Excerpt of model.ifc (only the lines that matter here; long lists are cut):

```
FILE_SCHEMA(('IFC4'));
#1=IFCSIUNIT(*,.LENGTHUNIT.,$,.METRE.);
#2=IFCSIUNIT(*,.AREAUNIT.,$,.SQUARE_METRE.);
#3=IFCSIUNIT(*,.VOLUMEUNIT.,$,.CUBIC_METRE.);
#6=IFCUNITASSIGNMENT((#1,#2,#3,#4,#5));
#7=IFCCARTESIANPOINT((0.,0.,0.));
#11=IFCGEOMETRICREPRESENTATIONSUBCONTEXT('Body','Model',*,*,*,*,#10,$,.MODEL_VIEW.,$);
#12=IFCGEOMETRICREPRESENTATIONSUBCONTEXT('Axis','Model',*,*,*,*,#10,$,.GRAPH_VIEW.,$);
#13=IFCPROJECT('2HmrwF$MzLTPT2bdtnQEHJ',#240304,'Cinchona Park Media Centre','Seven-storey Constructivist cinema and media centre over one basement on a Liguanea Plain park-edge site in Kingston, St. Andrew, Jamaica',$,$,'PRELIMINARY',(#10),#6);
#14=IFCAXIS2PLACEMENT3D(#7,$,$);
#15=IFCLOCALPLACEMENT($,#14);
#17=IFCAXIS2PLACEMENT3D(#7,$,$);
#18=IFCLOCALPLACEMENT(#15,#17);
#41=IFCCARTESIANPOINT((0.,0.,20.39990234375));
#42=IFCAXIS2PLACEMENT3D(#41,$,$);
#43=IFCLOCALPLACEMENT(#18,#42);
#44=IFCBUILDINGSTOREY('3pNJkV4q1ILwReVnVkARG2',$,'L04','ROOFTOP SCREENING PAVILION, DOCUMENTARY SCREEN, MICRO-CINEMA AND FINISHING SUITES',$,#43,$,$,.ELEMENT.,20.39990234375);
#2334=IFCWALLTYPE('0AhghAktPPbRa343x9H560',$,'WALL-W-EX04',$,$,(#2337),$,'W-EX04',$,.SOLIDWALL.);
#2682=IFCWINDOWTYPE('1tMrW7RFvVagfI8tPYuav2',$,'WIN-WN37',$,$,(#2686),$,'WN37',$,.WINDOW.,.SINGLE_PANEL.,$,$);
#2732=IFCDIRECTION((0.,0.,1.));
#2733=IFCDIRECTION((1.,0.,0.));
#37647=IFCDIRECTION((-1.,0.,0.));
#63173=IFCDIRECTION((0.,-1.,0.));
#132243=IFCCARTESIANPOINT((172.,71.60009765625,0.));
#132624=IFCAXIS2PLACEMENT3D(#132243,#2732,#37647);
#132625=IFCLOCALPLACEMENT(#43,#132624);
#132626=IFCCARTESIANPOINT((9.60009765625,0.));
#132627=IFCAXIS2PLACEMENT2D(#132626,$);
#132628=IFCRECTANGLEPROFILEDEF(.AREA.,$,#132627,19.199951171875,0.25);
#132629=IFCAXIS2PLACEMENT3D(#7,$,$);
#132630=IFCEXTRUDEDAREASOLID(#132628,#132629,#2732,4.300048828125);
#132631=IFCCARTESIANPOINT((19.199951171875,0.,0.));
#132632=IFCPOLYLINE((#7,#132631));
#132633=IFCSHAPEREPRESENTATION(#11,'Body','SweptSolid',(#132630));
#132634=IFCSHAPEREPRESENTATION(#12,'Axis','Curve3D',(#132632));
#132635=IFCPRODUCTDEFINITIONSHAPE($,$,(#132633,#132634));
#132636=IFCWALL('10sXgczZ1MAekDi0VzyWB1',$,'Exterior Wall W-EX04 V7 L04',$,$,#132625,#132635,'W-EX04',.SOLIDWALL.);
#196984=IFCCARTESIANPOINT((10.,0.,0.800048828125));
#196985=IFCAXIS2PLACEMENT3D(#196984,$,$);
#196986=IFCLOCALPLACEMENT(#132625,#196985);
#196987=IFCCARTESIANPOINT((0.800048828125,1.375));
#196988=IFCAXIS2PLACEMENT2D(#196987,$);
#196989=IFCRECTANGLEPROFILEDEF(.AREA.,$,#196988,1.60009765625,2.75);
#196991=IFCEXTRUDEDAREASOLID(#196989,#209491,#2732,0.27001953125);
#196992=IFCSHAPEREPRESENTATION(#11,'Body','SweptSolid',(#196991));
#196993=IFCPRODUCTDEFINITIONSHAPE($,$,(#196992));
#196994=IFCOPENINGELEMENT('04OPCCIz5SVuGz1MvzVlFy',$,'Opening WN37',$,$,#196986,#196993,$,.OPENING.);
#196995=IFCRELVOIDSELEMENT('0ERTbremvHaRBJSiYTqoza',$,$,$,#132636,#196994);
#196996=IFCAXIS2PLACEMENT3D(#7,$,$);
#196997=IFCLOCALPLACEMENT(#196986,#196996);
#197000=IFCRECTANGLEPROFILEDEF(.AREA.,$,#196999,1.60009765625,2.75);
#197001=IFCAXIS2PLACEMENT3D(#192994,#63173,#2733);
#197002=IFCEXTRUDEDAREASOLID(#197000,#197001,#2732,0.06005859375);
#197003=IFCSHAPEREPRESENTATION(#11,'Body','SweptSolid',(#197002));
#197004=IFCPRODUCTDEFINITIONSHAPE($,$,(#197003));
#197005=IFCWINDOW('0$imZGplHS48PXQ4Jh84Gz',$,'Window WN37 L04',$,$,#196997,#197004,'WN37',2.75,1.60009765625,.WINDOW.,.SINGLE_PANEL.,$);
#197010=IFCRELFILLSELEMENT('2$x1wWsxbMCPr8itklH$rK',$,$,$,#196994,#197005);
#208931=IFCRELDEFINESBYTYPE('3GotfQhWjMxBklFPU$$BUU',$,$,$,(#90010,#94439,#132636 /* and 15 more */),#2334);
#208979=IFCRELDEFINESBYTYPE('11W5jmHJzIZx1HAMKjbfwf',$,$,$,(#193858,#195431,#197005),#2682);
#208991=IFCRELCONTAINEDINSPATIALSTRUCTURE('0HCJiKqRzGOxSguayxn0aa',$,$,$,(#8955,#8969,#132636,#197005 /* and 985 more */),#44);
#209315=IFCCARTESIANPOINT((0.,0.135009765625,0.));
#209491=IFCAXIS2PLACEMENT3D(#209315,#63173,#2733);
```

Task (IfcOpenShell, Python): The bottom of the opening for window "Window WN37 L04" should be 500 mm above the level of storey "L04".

```python
import numpy as np
import ifcopenshell
import ifcopenshell.api.geometry
import ifcopenshell.geom
import ifcopenshell.util.element
import ifcopenshell.util.placement
import ifcopenshell.util.shape
import ifcopenshell.util.unit

model = ifcopenshell.open("model.ifc")
unit_scale = ifcopenshell.util.unit.calculate_unit_scale(model)

window = model.by_guid("0$imZGplHS48PXQ4Jh84Gz")
opening = window.FillsVoids[0].RelatingOpeningElement
storey = ifcopenshell.util.element.get_container(window, ifc_class="IfcBuildingStorey")
level = ifcopenshell.util.placement.get_local_placement(storey.ObjectPlacement)[2, 3]

# The opening's origin need not be at the sill, so measure its lowest point.
shape = ifcopenshell.geom.create_shape(ifcopenshell.geom.settings(), opening)
bottom = ifcopenshell.util.shape.get_shape_bottom_elevation(shape, shape.geometry) / unit_scale
dz = level + 0.5 / unit_scale - bottom

shift = np.array([0.0, 0.0, dz])
# The window is placed relative to its opening, so it follows when the opening moves.
matrix = ifcopenshell.util.placement.get_local_placement(opening.ObjectPlacement)
matrix[:3, 3] += shift
ifcopenshell.api.geometry.edit_object_placement(
    model, product=opening, matrix=matrix, is_si=False, should_transform_children=True
)

print(f"moved by {dz * unit_scale:+.3f} m")

model.write("model-out.ifc")
```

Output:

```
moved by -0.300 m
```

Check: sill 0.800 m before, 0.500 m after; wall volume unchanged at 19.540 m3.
